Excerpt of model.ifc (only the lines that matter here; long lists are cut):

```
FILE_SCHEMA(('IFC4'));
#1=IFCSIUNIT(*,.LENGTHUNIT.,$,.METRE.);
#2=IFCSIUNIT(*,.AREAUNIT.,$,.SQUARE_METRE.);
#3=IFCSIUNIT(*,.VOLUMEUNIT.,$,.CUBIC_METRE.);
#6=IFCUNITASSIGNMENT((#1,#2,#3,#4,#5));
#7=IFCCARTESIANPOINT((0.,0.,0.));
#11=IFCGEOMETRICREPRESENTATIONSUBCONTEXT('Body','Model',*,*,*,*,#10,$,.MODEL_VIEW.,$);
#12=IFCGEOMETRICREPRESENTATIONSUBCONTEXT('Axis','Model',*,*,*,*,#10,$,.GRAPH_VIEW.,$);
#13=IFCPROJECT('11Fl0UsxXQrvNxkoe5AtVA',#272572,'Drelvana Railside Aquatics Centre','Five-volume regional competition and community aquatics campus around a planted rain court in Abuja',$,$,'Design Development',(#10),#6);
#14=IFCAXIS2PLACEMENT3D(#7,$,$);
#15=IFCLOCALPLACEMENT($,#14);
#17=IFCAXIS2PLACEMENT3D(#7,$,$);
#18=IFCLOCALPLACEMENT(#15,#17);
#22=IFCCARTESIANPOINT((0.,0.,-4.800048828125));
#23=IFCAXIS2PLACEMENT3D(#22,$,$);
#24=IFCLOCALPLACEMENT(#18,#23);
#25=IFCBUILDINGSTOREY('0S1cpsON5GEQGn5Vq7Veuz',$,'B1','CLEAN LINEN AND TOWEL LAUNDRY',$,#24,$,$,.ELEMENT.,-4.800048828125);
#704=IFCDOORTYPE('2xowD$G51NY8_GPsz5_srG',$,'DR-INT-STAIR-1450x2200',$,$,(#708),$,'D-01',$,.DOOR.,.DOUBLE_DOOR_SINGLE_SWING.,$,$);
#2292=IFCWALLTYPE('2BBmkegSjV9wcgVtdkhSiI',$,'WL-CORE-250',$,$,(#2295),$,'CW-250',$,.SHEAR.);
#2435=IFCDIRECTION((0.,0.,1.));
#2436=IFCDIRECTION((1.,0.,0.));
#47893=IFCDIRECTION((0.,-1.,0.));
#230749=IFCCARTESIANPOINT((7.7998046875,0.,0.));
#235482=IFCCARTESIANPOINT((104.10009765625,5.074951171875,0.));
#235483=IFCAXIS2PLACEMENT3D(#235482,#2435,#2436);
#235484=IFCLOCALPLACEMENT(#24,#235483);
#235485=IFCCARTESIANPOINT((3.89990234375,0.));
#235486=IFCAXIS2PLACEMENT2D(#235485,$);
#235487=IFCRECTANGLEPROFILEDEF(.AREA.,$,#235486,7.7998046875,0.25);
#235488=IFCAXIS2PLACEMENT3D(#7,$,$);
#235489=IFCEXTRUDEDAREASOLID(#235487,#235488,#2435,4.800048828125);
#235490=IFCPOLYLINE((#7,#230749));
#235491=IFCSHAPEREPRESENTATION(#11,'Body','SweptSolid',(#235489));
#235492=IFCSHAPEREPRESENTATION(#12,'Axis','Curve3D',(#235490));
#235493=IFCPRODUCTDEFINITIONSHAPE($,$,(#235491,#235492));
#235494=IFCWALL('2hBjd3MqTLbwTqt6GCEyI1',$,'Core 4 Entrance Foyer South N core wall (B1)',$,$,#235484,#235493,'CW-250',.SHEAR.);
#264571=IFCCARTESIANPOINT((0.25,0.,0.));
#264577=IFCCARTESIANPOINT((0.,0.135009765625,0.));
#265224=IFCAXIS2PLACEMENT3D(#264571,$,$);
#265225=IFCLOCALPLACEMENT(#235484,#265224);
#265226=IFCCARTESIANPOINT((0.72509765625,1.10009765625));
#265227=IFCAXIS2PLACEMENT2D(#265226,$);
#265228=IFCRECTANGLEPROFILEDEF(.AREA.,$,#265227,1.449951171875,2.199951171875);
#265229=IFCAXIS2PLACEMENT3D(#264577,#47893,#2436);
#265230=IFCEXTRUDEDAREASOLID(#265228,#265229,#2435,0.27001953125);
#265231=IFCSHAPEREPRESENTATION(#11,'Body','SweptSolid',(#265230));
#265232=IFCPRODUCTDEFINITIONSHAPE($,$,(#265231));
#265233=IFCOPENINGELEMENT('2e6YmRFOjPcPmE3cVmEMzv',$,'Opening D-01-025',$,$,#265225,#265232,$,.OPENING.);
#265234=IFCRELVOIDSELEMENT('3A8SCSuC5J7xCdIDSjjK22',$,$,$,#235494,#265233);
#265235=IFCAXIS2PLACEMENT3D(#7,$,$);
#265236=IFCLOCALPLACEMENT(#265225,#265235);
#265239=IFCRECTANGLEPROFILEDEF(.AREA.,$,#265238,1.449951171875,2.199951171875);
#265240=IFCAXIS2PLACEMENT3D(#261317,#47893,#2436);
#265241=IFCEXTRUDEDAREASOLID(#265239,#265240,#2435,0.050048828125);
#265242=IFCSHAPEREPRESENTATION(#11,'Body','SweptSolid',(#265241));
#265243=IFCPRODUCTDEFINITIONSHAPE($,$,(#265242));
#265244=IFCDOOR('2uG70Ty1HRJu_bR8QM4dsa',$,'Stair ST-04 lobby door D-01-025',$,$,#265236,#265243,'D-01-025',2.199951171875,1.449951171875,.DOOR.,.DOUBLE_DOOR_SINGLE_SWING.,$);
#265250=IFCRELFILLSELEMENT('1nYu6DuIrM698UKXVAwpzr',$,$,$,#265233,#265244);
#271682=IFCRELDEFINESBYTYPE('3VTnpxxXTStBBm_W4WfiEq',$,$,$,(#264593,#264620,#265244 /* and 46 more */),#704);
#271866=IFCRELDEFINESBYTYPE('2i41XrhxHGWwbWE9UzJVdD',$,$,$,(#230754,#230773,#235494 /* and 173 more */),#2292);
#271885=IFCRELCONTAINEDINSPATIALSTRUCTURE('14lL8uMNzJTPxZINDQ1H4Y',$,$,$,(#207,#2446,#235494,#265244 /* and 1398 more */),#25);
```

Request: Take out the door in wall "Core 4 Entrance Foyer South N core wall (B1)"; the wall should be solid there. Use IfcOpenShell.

```python
import ifcopenshell
import ifcopenshell.api.feature
import ifcopenshell.api.root
import ifcopenshell.geom
import ifcopenshell.util.shape

model = ifcopenshell.open("model.ifc")
settings = ifcopenshell.geom.settings()


def volume(element):
    """Net volume in cubic metres, openings subtracted."""
    shape = ifcopenshell.geom.create_shape(settings, element)
    return ifcopenshell.util.shape.get_volume(shape.geometry)


door = model.by_guid("2uG70Ty1HRJu_bR8QM4dsa")
opening = door.FillsVoids[0].RelatingOpeningElement
wall = opening.VoidsElements[0].RelatingBuildingElement
before = volume(wall)

ifcopenshell.api.root.remove_product(model, product=door)
ifcopenshell.api.feature.remove_feature(model, feature=opening)

after = volume(wall)

print(f"wall volume {before:.3f} -> {after:.3f} m3")

model.write("model-out.ifc")
```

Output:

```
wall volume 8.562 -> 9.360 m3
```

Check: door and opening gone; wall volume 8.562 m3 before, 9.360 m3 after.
